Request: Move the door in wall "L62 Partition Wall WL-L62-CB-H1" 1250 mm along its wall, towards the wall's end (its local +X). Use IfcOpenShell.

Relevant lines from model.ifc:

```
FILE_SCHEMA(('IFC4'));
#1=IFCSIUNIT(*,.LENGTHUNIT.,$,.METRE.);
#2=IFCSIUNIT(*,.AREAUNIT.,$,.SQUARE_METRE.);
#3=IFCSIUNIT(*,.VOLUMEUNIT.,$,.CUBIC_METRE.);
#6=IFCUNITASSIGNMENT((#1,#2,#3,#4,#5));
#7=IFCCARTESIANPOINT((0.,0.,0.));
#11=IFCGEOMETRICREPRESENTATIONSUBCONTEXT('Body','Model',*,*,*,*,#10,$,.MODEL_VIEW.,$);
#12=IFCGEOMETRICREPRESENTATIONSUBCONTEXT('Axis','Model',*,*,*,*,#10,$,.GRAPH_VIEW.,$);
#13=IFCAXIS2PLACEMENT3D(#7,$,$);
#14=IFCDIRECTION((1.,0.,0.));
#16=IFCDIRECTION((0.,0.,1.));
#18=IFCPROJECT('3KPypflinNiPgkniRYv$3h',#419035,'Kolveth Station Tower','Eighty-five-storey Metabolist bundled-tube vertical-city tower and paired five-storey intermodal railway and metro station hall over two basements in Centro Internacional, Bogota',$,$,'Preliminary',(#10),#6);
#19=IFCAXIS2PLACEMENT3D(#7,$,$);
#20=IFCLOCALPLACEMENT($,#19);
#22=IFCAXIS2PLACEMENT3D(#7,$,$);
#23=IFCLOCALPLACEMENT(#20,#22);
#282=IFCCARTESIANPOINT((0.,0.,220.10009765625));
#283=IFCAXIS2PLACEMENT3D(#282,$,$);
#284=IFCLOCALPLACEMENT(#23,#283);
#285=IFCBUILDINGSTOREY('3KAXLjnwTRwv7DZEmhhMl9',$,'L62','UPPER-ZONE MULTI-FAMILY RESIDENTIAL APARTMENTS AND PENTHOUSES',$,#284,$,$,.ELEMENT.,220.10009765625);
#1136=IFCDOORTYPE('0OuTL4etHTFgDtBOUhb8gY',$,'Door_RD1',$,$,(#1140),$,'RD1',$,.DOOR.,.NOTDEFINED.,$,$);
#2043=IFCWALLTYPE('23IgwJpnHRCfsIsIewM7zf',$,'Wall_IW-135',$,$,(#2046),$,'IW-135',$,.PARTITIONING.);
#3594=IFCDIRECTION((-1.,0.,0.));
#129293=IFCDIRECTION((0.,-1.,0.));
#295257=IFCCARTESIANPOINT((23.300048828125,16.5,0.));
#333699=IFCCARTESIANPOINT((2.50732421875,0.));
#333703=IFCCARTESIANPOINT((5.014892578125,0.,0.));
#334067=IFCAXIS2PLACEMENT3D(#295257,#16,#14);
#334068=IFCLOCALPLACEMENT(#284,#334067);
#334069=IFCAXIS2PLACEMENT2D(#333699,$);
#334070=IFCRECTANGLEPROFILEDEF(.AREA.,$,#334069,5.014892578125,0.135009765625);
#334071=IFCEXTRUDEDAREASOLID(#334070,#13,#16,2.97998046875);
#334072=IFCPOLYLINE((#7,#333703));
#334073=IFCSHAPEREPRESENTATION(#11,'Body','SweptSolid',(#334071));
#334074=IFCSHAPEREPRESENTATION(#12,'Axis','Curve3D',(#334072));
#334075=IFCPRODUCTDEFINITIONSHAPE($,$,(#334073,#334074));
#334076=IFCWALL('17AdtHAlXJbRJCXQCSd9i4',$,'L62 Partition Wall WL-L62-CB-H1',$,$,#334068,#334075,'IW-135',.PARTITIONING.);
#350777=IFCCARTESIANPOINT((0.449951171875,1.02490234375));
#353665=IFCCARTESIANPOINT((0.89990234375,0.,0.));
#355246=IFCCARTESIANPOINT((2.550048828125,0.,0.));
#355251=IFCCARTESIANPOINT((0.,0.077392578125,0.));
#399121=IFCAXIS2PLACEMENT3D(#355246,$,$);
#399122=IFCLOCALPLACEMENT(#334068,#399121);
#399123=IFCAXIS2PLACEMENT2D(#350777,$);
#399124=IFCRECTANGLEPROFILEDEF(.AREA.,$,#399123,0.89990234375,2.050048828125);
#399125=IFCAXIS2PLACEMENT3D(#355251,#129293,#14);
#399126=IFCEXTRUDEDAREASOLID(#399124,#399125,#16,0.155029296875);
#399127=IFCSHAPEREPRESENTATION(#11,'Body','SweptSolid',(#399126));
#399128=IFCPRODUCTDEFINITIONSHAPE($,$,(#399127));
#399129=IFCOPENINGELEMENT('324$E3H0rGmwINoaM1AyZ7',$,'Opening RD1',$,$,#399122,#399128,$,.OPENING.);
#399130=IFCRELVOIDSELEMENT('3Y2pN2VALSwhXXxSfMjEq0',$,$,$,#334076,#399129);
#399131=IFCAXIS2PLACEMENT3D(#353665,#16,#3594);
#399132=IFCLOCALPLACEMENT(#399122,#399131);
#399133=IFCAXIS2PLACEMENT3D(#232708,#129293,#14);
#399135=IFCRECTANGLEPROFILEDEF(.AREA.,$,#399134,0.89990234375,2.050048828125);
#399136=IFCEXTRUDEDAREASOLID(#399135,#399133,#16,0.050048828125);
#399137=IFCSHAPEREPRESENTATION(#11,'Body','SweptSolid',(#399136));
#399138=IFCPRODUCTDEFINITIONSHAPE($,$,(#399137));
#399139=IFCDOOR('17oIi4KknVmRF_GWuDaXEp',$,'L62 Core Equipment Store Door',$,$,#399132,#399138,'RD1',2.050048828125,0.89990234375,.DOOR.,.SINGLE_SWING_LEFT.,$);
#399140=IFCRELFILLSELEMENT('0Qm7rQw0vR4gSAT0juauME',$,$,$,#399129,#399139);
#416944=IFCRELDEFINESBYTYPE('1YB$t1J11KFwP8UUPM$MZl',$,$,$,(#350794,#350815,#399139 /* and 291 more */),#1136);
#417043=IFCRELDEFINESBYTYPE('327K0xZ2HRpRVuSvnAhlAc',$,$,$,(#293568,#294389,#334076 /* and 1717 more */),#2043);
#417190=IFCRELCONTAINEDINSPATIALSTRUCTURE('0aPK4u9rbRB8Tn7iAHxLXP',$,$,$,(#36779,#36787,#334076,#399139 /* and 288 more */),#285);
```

```python
import ifcopenshell
import ifcopenshell.api.geometry
import ifcopenshell.util.placement
import ifcopenshell.util.unit

model = ifcopenshell.open("model.ifc")
unit_scale = ifcopenshell.util.unit.calculate_unit_scale(model)

door = model.by_guid("17oIi4KknVmRF_GWuDaXEp")
opening = door.FillsVoids[0].RelatingOpeningElement
wall = opening.VoidsElements[0].RelatingBuildingElement

wall_matrix = ifcopenshell.util.placement.get_local_placement(wall.ObjectPlacement)
shift = wall_matrix[:3, 0] * 1.25 / unit_scale
before = ifcopenshell.util.placement.get_local_placement(door.ObjectPlacement)[:3, 3].copy()

# The door is placed relative to its opening, so it follows when the opening moves.
matrix = ifcopenshell.util.placement.get_local_placement(opening.ObjectPlacement)
matrix[:3, 3] += shift
ifcopenshell.api.geometry.edit_object_placement(
    model, product=opening, matrix=matrix, is_si=False, should_transform_children=True
)

after = ifcopenshell.util.placement.get_local_placement(door.ObjectPlacement)[:3, 3]
print("door moved by", (after - before).round(3) + 0.0)

model.write("model-out.ifc")
```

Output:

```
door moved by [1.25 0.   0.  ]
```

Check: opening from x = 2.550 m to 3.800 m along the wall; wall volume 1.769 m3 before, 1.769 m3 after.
